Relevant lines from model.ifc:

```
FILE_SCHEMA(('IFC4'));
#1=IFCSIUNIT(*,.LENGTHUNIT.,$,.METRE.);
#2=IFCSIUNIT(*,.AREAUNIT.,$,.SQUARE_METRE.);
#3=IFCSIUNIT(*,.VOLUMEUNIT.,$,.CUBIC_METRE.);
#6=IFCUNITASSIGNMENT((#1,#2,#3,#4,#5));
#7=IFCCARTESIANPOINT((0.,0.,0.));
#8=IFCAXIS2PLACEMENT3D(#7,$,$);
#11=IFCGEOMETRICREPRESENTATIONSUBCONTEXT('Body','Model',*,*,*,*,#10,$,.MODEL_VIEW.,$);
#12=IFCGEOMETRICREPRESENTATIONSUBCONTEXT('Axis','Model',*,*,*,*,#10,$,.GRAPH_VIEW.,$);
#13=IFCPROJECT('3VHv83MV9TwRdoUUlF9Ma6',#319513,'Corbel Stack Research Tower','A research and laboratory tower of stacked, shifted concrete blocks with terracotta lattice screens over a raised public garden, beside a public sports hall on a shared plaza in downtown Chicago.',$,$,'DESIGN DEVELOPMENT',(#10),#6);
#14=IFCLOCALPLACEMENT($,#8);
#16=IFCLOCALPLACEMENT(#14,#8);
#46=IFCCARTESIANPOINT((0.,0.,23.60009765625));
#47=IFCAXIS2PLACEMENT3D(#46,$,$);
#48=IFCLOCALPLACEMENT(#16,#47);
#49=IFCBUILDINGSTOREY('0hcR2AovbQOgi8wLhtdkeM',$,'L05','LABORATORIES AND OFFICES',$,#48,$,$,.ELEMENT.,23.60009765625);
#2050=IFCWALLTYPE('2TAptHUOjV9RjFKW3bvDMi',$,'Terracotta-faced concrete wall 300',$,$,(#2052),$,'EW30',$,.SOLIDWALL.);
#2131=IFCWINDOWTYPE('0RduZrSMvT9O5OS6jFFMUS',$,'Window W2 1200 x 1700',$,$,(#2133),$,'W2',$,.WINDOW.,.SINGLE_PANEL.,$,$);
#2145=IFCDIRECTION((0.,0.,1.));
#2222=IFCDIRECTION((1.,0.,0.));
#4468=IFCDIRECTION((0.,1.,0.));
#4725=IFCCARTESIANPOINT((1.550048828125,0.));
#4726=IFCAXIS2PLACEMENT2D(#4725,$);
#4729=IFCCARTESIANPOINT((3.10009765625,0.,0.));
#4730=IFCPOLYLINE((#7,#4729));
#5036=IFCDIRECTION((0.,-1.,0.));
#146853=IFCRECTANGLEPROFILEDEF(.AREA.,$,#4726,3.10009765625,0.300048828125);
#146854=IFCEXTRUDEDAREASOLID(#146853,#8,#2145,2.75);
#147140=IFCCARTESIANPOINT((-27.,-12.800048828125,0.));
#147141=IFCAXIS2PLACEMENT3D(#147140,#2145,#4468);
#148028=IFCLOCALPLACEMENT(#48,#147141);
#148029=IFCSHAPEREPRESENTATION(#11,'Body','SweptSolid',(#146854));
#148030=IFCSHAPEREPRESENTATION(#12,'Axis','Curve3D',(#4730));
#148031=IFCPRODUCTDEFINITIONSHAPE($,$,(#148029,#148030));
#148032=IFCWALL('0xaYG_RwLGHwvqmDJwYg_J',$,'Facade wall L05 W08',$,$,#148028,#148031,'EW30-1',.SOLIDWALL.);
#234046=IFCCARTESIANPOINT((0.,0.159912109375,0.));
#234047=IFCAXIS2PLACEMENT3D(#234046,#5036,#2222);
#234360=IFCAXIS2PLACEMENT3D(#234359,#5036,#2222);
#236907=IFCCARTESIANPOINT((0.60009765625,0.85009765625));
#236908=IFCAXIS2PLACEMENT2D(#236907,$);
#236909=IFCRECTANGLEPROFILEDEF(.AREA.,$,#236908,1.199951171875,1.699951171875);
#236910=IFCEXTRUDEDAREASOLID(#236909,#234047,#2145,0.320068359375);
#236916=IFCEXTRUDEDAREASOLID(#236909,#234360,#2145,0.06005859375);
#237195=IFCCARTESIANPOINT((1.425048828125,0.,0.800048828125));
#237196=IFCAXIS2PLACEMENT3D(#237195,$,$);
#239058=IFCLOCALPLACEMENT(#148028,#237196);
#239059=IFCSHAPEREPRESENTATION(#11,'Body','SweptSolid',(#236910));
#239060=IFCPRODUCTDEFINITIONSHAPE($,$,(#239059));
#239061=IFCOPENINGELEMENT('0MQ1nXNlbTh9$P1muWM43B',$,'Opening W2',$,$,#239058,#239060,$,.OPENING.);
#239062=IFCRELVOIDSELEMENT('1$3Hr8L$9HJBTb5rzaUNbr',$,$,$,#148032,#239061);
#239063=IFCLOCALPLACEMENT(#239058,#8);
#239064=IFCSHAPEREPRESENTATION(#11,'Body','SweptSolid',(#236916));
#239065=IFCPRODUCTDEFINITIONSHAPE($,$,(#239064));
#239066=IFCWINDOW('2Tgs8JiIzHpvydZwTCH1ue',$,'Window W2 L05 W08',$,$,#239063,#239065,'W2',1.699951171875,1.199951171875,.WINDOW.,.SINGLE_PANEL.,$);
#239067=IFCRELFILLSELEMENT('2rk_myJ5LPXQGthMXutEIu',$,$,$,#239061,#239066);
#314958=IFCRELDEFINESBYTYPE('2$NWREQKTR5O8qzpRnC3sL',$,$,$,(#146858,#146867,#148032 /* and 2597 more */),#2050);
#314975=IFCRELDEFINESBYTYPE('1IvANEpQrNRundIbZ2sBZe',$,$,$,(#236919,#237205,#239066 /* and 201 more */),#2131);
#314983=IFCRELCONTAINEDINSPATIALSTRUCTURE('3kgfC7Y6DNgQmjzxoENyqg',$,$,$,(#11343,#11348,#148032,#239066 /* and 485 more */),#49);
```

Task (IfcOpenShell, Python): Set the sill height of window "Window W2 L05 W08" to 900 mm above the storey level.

```python
import numpy as np
import ifcopenshell
import ifcopenshell.api.geometry
import ifcopenshell.geom
import ifcopenshell.util.element
import ifcopenshell.util.placement
import ifcopenshell.util.shape
import ifcopenshell.util.unit

model = ifcopenshell.open("model.ifc")
unit_scale = ifcopenshell.util.unit.calculate_unit_scale(model)

window = model.by_guid("2Tgs8JiIzHpvydZwTCH1ue")
opening = window.FillsVoids[0].RelatingOpeningElement
storey = ifcopenshell.util.element.get_container(window, ifc_class="IfcBuildingStorey")
level = ifcopenshell.util.placement.get_local_placement(storey.ObjectPlacement)[2, 3]

# The opening's origin need not be at the sill, so measure its lowest point.
shape = ifcopenshell.geom.create_shape(ifcopenshell.geom.settings(), opening)
bottom = ifcopenshell.util.shape.get_shape_bottom_elevation(shape, shape.geometry) / unit_scale
dz = level + 0.9 - bottom

shift = np.array([0.0, 0.0, dz])
# The window is placed relative to its opening, so it follows when the opening moves.
matrix = ifcopenshell.util.placement.get_local_placement(opening.ObjectPlacement)
matrix[:3, 3] += shift
ifcopenshell.api.geometry.edit_object_placement(
    model, product=opening, matrix=matrix, is_si=False, should_transform_children=True
)

print(f"moved by {dz * unit_scale:+.3f} m")

model.write("model-out.ifc")
```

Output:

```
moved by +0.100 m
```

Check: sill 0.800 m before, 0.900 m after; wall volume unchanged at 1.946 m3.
